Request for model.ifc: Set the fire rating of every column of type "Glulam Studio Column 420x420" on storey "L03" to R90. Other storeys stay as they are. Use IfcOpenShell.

First a look at what the model holds.

```python
import ifcopenshell
import ifcopenshell.util.element

model = ifcopenshell.open("model.ifc")
print(model.schema)
storey = next(s for s in model.by_type("IfcBuildingStorey") if s.Name == "L03")
columns = [e for e in ifcopenshell.util.element.get_decomposition(storey) if e.is_a("IfcColumn")]
seen = {}
for e in columns:
    element_type = ifcopenshell.util.element.get_type(e)
    key = (element_type.Name if element_type != e and element_type else None, ifcopenshell.util.element.get_pset(e, "Pset_ColumnCommon", "FireRating"))
    seen[key] = seen.get(key, 0) + 1
for (name, value), count in sorted(seen.items(), key=str):
    print(count, "x", name, "|", value)
```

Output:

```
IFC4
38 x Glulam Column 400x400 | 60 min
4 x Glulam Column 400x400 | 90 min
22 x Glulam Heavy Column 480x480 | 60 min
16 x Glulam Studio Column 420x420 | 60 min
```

```python
import ifcopenshell
import ifcopenshell.api.pset
import ifcopenshell.util.element

model = ifcopenshell.open("model.ifc")

storey = next(s for s in model.by_type("IfcBuildingStorey") if s.Name == "L03")
columns = [e for e in ifcopenshell.util.element.get_decomposition(storey) if e.is_a("IfcColumn")]

count = 0
for e in columns:
    element_type = ifcopenshell.util.element.get_type(e)
    if element_type in (None, e) or element_type.Name != "Glulam Studio Column 420x420":
        continue
    # add_pset returns the element's existing set when there is one.
    pset = ifcopenshell.api.pset.add_pset(model, product=e, name="Pset_ColumnCommon")
    ifcopenshell.api.pset.edit_pset(model, pset=pset, properties={"FireRating": "R90"})
    count += 1

print(count, "columns updated")

model.write("model-out.ifc")
```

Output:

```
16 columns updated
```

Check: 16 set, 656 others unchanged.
